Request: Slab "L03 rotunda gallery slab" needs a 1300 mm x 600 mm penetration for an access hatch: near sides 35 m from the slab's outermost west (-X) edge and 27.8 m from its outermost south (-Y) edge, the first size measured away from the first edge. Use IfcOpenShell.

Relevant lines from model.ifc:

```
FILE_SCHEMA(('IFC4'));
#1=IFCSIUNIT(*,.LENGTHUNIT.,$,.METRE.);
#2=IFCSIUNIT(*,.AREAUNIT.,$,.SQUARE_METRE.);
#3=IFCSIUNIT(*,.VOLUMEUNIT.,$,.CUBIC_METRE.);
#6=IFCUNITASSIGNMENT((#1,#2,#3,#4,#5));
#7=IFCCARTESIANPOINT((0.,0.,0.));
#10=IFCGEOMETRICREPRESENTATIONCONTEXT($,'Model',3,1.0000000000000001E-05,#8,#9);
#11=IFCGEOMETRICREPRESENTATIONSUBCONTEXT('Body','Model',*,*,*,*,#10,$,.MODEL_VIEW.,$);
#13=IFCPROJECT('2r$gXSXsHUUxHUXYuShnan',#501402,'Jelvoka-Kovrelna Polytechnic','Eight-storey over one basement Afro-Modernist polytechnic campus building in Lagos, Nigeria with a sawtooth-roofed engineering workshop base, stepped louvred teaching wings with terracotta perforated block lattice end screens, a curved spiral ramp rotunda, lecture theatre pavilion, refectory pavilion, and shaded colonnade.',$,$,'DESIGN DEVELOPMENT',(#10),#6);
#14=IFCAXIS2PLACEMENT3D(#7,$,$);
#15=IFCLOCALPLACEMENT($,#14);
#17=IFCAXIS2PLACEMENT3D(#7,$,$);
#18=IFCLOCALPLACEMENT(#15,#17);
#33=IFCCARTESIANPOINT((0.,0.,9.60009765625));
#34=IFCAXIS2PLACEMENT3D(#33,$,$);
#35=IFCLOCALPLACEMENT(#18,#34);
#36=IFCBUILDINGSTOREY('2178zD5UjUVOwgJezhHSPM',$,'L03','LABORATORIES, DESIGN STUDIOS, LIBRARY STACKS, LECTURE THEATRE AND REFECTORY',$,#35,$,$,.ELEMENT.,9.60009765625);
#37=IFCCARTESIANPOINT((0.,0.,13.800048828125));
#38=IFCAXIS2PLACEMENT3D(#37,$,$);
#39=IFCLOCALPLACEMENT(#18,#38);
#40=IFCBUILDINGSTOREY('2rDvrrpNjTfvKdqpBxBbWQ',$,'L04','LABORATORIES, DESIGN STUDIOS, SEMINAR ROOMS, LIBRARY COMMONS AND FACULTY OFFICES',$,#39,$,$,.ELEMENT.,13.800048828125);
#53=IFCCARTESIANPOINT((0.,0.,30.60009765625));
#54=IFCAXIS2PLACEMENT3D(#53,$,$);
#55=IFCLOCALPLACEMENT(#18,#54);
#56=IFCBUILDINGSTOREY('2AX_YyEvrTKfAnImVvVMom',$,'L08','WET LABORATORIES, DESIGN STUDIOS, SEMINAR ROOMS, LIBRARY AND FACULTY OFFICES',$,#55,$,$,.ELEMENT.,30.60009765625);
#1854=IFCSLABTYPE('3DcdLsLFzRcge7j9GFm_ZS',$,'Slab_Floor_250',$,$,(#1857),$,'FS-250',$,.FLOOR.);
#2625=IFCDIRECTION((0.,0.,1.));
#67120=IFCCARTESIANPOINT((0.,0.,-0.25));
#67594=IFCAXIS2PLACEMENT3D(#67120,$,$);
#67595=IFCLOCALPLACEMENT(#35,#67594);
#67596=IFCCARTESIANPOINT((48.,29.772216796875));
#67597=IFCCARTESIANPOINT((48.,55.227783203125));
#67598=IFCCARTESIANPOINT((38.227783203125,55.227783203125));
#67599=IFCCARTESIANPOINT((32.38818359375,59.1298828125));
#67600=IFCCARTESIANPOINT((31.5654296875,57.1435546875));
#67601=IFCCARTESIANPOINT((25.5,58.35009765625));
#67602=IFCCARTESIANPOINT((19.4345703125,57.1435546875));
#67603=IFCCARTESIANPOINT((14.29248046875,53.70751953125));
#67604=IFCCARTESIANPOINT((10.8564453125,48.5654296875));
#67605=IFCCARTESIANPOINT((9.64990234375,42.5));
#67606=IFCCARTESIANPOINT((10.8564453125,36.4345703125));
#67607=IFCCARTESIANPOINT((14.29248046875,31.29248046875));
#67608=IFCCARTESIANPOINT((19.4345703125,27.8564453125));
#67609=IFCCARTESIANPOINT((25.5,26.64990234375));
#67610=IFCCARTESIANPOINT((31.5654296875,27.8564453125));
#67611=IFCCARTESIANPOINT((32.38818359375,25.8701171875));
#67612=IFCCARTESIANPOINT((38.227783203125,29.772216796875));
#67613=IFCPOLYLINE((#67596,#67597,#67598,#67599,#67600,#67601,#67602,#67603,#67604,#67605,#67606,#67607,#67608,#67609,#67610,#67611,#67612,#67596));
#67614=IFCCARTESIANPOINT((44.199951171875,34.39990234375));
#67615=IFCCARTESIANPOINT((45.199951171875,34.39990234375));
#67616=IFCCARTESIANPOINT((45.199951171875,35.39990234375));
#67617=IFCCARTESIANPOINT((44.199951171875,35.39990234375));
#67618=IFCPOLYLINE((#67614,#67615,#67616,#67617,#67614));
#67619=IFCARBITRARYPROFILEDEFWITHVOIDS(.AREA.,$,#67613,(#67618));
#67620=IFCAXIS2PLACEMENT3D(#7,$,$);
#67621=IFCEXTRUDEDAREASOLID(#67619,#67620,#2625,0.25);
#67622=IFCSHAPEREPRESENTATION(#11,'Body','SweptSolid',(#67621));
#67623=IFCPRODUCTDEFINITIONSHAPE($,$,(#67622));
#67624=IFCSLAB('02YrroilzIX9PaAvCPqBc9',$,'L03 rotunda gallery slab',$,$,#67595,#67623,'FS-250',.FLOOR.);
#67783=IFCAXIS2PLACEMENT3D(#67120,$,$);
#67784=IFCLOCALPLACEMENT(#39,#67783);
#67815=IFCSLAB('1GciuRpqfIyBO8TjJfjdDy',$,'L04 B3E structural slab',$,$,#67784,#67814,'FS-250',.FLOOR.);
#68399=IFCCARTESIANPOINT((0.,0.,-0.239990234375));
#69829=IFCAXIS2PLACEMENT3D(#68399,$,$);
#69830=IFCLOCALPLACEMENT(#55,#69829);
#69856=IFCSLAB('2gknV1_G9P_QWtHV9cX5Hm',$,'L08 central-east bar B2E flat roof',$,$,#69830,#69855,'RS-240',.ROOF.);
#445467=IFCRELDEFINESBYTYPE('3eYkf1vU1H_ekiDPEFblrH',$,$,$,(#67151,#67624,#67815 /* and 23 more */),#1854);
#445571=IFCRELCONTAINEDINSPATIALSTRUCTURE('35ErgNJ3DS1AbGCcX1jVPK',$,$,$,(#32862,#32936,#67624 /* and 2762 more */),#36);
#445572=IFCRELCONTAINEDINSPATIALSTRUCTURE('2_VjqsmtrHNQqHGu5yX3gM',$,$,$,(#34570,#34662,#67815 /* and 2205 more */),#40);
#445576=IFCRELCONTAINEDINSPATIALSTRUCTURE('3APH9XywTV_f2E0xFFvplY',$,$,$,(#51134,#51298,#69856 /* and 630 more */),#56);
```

```python
import numpy as np
import ifcopenshell
import ifcopenshell.api.feature
import ifcopenshell.api.geometry
import ifcopenshell.api.root
import ifcopenshell.geom
import ifcopenshell.util.placement
import ifcopenshell.util.representation
import ifcopenshell.util.shape
import ifcopenshell.util.unit

model = ifcopenshell.open("model.ifc")
unit_scale = ifcopenshell.util.unit.calculate_unit_scale(model)
settings = ifcopenshell.geom.settings()


def volume(element):
    """Net volume in cubic metres, openings subtracted."""
    shape = ifcopenshell.geom.create_shape(settings, element)
    return ifcopenshell.util.shape.get_volume(shape.geometry)


slab = model.by_guid("02YrroilzIX9PaAvCPqBc9")
before = volume(slab)

# Extent in the slab's own axes, in metres. The edges named are its -X and -Y sides.
slab_shape = ifcopenshell.geom.create_shape(settings, slab)
vertices = ifcopenshell.util.shape.get_vertices(slab_shape.geometry)
x_min, y_min, bottom = vertices.min(axis=0)
top = vertices[:, 2].max()

opening = ifcopenshell.api.root.create_entity(model, ifc_class="IfcOpeningElement", name="Access hatch opening", predefined_type="OPENING")
context = ifcopenshell.util.representation.get_context(model, "Model", "Body", "MODEL_VIEW")
width, depth = 1.3, 0.6
outline = [(0.0, 0.0), (width, 0.0), (width, depth), (0.0, depth), (0.0, 0.0)]
# Overshoot both faces by 50 mm so the cut is clean.
shape = ifcopenshell.api.geometry.add_slab_representation(
    model, context=context, depth=top - bottom + 0.1, polyline=outline
)
ifcopenshell.api.geometry.assign_representation(model, product=opening, representation=shape)

matrix = ifcopenshell.util.placement.get_local_placement(slab.ObjectPlacement)
matrix[:, 3] = matrix @ np.append(np.array([x_min + 35, y_min + 27.8, bottom - 0.05]) / unit_scale, 1.0)
ifcopenshell.api.geometry.edit_object_placement(model, product=opening, matrix=matrix, is_si=False)
ifcopenshell.api.feature.add_feature(model, feature=opening, element=slab)

after = volume(slab)

print(f"slab volume {before:.3f} -> {after:.3f} m3")

model.write("model_rev.ifc")
```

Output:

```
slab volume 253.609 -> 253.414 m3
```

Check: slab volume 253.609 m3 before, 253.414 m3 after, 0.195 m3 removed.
